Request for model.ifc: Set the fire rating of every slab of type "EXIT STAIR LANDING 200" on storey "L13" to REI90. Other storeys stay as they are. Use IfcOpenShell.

First a look at what the model holds.

```python
import ifcopenshell
import ifcopenshell.util.element

model = ifcopenshell.open("model.ifc")
print(model.schema)
storey = next(s for s in model.by_type("IfcBuildingStorey") if s.Name == "L13")
slabs = [e for e in ifcopenshell.util.element.get_decomposition(storey) if e.is_a("IfcSlab")]
seen = {}
for e in slabs:
    element_type = ifcopenshell.util.element.get_type(e)
    key = (element_type.Name if element_type != e and element_type else None, ifcopenshell.util.element.get_pset(e, "Pset_SlabCommon", "FireRating"))
    seen[key] = seen.get(key, 0) + 1
for (name, value), count in sorted(seen.items(), key=str):
    print(count, "x", name, "|", value)
```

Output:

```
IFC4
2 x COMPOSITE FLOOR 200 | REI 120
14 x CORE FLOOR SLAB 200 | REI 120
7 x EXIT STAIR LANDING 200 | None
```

```python
import ifcopenshell
import ifcopenshell.api.pset
import ifcopenshell.util.element

model = ifcopenshell.open("model.ifc")

storey = next(s for s in model.by_type("IfcBuildingStorey") if s.Name == "L13")
slabs = [e for e in ifcopenshell.util.element.get_decomposition(storey) if e.is_a("IfcSlab")]

count = 0
for e in slabs:
    element_type = ifcopenshell.util.element.get_type(e)
    if element_type in (None, e) or element_type.Name != "EXIT STAIR LANDING 200":
        continue
    found = ifcopenshell.util.element.get_pset(e, "Pset_SlabCommon", should_inherit=False)
    if found:
        pset = model.by_id(found["id"])
        if len(ifcopenshell.util.element.get_elements_by_pset(pset)) > 1:
            pset = ifcopenshell.api.pset.unshare_pset(model, products=[e], pset=pset)[0]
    else:
        pset = ifcopenshell.api.pset.add_pset(model, product=e, name="Pset_SlabCommon")
    ifcopenshell.api.pset.edit_pset(model, pset=pset, properties={"FireRating": "REI90"})
    count += 1

print(count, "slabs updated")

model.write("model_v2.ifc")
```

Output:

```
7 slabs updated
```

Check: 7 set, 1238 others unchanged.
